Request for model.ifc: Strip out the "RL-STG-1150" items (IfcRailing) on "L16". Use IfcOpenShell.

First a look at what the model holds.

```python
import ifcopenshell
import ifcopenshell.util.element

model = ifcopenshell.open("model.ifc")
print(model.schema)
storey = next(s for s in model.by_type("IfcBuildingStorey") if s.Name == "L16")
railings = [e for e in ifcopenshell.util.element.get_decomposition(storey) if e.is_a("IfcRailing")]
seen = {}
for e in railings:
    element_type = ifcopenshell.util.element.get_type(e)
    name = element_type.Name if element_type not in (None, e) else None
    seen[name] = seen.get(name, 0) + 1
for name, count in sorted(seen.items(), key=str):
    print(count, "x", name)
```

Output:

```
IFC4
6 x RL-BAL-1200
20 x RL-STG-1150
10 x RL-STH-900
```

```python
import ifcopenshell
import ifcopenshell.api.root
import ifcopenshell.util.element

model = ifcopenshell.open("model.ifc")

storey = next(s for s in model.by_type("IfcBuildingStorey") if s.Name == "L16")
railings = [e for e in ifcopenshell.util.element.get_decomposition(storey) if e.is_a("IfcRailing")]
targets = [e for e in railings if (t := ifcopenshell.util.element.get_type(e)) not in (None, e) and t.Name == "RL-STG-1150"]

for e in targets:
    ifcopenshell.api.root.remove_product(model, product=e)
print(len(targets), "removed")

model.write("model_rev.ifc")
```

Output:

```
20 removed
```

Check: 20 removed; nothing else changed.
